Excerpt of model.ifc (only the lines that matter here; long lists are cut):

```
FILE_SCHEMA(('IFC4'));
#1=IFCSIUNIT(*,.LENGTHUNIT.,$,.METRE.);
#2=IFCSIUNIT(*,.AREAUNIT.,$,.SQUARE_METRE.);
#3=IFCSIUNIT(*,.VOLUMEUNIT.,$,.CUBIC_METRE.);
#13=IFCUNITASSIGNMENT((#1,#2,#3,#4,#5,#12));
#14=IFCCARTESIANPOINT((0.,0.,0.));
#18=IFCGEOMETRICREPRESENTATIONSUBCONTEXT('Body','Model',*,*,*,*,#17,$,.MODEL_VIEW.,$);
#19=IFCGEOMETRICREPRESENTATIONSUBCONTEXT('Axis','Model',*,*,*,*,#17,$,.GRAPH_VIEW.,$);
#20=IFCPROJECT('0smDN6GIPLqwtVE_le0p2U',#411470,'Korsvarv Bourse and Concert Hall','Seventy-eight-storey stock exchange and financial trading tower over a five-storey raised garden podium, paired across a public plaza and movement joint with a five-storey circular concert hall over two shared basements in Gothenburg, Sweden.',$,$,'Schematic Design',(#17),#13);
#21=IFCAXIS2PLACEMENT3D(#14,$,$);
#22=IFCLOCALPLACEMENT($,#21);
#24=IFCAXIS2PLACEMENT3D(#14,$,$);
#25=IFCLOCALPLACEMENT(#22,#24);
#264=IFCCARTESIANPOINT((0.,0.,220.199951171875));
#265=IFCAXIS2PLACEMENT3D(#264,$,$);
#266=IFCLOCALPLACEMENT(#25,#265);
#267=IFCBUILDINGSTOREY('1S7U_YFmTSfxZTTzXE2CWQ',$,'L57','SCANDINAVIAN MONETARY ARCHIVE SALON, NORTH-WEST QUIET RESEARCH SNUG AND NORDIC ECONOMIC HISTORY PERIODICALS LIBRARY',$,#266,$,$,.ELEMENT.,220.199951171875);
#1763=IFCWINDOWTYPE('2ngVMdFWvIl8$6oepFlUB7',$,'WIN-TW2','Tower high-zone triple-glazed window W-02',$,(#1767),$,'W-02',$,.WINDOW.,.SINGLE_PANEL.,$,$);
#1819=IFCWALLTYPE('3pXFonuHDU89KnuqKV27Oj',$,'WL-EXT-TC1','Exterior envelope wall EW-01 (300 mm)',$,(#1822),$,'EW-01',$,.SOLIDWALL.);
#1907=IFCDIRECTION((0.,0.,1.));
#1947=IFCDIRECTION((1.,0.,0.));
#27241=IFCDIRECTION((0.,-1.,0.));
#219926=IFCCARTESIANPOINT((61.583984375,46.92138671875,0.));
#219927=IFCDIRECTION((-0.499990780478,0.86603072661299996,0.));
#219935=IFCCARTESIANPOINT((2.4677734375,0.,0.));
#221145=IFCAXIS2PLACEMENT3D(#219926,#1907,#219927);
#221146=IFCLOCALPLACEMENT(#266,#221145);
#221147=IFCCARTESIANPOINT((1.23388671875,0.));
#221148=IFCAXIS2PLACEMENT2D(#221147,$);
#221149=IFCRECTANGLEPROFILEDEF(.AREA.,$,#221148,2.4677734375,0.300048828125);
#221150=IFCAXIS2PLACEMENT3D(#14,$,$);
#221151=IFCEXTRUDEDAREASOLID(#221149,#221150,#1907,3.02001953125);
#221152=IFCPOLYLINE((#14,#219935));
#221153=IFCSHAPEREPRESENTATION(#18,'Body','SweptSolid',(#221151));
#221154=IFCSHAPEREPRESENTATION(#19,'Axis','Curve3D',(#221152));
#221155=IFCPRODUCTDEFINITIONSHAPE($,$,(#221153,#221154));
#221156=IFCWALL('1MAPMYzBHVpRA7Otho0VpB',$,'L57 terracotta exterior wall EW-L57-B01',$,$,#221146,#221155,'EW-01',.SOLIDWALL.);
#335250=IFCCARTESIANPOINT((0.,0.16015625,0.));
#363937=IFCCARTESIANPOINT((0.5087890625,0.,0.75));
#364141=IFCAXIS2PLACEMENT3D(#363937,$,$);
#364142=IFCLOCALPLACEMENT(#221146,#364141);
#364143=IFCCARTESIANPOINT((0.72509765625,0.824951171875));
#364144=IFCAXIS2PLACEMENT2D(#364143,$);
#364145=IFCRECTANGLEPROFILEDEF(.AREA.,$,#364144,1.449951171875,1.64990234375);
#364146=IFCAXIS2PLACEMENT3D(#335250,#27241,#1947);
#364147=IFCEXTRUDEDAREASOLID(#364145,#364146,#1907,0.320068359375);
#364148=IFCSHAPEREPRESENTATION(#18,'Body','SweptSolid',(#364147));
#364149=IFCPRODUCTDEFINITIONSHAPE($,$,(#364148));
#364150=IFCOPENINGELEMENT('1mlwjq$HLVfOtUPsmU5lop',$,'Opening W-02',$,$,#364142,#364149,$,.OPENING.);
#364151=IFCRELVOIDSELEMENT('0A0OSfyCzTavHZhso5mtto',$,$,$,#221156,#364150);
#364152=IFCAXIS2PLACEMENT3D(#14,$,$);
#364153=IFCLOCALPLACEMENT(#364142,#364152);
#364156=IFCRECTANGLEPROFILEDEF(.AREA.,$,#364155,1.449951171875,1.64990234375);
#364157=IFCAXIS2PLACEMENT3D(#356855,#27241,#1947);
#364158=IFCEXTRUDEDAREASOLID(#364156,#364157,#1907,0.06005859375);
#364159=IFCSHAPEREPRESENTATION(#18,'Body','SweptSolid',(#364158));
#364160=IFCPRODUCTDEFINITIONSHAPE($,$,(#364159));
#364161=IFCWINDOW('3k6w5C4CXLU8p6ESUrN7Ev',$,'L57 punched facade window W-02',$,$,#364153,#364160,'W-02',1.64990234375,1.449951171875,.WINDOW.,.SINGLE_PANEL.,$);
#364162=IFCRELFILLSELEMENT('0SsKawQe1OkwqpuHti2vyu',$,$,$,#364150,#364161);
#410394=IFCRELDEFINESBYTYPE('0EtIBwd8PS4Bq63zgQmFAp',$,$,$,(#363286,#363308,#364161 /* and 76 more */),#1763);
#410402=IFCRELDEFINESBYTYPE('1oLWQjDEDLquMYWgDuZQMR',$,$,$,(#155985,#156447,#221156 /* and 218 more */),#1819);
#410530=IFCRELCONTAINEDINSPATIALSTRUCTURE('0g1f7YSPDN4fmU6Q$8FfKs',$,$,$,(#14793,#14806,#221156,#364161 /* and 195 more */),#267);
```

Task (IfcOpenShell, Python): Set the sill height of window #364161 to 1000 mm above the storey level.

```python
import numpy as np
import ifcopenshell
import ifcopenshell.api.geometry
import ifcopenshell.geom
import ifcopenshell.util.element
import ifcopenshell.util.placement
import ifcopenshell.util.shape
import ifcopenshell.util.unit

model = ifcopenshell.open("model.ifc")
unit_scale = ifcopenshell.util.unit.calculate_unit_scale(model)

window = model.by_guid("3k6w5C4CXLU8p6ESUrN7Ev")
opening = window.FillsVoids[0].RelatingOpeningElement
storey = ifcopenshell.util.element.get_container(window, ifc_class="IfcBuildingStorey")
level = ifcopenshell.util.placement.get_local_placement(storey.ObjectPlacement)[2, 3]

# The opening's origin need not be at the sill, so measure its lowest point.
shape = ifcopenshell.geom.create_shape(ifcopenshell.geom.settings(), opening)
bottom = ifcopenshell.util.shape.get_shape_bottom_elevation(shape, shape.geometry) / unit_scale
dz = level + 1 / unit_scale - bottom

shift = np.array([0.0, 0.0, dz])
# The window is placed relative to its opening, so it follows when the opening moves.
matrix = ifcopenshell.util.placement.get_local_placement(opening.ObjectPlacement)
matrix[:3, 3] += shift
ifcopenshell.api.geometry.edit_object_placement(
    model, product=opening, matrix=matrix, is_si=False, should_transform_children=True
)

print(f"moved by {dz * unit_scale:+.3f} m")

model.write("model_updated.ifc")
```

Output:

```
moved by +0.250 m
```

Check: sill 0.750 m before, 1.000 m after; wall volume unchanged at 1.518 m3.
